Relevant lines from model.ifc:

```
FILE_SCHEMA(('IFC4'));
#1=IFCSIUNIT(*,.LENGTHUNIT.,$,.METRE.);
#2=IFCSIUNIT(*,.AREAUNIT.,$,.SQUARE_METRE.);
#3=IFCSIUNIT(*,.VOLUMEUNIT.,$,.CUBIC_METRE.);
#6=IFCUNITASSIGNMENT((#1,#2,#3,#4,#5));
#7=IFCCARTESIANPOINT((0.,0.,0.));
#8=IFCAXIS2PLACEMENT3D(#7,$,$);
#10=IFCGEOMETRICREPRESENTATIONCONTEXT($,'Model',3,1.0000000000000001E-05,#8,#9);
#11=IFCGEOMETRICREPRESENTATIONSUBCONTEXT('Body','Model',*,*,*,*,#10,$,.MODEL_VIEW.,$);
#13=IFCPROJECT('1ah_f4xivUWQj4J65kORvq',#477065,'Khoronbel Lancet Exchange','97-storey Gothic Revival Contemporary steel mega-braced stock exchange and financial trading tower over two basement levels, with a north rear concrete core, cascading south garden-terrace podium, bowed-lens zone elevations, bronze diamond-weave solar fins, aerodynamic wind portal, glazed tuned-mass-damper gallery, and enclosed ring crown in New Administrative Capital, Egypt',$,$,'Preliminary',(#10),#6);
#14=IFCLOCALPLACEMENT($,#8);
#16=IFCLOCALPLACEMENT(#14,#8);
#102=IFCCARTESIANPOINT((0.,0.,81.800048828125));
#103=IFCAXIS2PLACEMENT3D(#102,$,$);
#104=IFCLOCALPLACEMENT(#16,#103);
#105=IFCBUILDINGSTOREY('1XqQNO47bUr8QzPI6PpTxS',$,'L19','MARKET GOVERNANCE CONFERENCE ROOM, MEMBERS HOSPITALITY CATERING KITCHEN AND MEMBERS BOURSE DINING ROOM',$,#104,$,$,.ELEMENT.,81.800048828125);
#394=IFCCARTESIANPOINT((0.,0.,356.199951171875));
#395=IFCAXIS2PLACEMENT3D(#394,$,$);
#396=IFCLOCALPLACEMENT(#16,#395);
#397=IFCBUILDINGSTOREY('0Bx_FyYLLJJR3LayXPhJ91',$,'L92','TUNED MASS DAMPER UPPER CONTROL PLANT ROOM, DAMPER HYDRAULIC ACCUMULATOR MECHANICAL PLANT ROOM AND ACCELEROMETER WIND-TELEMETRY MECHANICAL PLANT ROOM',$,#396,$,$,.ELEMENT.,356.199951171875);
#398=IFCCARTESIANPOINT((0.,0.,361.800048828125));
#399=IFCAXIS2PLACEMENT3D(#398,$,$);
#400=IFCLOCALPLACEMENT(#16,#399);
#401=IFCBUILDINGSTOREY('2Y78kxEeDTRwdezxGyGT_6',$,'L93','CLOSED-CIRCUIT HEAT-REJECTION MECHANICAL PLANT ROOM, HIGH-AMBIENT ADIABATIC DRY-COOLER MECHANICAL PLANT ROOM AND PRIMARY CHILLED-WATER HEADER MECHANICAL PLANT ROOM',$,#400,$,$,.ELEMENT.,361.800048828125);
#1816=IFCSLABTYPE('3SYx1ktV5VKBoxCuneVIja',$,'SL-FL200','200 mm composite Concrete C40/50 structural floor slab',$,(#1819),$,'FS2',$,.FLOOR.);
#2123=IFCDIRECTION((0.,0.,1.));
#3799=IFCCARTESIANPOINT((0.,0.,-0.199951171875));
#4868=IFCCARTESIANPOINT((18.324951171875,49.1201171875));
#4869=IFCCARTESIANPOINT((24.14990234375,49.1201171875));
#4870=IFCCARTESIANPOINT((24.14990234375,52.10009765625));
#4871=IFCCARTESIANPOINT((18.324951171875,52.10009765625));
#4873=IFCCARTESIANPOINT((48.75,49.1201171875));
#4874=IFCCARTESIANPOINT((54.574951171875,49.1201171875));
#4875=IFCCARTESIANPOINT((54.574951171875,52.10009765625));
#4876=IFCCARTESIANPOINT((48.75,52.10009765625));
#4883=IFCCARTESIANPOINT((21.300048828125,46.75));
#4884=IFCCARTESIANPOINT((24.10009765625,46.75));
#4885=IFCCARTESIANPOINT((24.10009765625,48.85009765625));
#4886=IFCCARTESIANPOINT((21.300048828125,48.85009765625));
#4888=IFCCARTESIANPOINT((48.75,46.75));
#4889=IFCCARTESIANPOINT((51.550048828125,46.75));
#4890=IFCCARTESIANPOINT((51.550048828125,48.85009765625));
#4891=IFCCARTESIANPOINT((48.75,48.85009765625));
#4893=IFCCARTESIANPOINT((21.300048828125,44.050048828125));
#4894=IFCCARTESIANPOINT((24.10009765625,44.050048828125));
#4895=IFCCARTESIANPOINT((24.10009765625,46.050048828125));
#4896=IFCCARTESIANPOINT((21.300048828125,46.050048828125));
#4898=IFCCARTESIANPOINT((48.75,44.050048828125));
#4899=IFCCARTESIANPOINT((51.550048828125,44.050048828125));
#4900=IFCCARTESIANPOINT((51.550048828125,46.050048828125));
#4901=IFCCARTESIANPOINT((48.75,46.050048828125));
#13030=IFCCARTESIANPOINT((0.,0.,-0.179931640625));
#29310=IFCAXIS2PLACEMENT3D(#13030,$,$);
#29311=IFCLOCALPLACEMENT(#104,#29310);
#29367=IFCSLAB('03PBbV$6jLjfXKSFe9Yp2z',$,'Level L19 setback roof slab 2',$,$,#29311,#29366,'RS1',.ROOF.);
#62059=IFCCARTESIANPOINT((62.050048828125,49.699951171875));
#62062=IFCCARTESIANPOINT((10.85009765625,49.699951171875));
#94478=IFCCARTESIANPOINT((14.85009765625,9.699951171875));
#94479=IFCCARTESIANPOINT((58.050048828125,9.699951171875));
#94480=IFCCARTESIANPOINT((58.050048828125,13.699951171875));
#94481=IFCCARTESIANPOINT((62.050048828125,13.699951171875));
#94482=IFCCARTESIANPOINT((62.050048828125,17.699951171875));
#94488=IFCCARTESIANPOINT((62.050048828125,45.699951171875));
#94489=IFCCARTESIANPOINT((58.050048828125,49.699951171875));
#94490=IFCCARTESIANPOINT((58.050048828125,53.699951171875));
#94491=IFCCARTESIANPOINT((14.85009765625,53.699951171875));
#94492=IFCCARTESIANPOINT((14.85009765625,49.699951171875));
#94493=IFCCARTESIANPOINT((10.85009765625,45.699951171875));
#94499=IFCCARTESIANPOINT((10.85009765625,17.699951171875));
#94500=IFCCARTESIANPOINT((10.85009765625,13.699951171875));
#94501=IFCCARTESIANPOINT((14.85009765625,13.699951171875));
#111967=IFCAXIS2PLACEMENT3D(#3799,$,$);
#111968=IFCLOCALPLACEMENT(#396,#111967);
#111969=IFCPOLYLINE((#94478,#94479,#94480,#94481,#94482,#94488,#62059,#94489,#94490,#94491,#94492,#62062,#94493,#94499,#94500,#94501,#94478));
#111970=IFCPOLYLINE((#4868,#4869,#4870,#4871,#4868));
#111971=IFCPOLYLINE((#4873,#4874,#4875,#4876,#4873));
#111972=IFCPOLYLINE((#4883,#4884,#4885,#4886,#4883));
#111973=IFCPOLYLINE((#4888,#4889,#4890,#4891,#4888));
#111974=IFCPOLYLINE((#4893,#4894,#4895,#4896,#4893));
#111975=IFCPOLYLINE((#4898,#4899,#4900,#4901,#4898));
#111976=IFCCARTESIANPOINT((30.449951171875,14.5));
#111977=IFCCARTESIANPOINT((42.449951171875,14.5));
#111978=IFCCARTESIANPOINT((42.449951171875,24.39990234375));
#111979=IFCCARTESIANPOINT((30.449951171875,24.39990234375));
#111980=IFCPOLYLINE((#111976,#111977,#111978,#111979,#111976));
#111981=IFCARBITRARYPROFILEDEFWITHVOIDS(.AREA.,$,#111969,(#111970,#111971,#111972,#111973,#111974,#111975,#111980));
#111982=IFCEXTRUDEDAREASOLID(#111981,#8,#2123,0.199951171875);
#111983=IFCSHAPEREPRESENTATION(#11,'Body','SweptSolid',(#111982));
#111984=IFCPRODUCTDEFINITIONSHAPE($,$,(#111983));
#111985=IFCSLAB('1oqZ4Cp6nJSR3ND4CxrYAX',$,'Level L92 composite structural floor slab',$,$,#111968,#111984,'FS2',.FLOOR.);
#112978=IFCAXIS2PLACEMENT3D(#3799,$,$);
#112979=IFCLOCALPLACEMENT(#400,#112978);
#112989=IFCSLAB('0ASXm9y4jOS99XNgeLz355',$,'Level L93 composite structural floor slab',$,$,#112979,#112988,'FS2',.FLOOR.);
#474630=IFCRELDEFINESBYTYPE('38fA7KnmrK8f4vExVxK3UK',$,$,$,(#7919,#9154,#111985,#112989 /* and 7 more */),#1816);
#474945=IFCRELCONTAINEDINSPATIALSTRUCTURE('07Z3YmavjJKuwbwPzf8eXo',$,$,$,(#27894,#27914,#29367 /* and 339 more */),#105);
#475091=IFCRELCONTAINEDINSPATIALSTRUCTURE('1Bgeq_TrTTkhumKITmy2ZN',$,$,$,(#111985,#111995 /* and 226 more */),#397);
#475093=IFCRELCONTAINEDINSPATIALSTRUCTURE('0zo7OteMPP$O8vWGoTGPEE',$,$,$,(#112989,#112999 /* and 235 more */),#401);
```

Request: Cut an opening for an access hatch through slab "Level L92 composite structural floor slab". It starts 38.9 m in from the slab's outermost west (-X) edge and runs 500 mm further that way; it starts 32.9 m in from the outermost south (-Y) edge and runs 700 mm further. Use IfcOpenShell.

```python
import numpy as np
import ifcopenshell
import ifcopenshell.api.feature
import ifcopenshell.api.geometry
import ifcopenshell.api.root
import ifcopenshell.geom
import ifcopenshell.util.placement
import ifcopenshell.util.representation
import ifcopenshell.util.shape
import ifcopenshell.util.unit

model = ifcopenshell.open("model.ifc")
unit_scale = ifcopenshell.util.unit.calculate_unit_scale(model)
settings = ifcopenshell.geom.settings()


def volume(element):
    """Net volume in cubic metres, openings subtracted."""
    shape = ifcopenshell.geom.create_shape(settings, element)
    return ifcopenshell.util.shape.get_volume(shape.geometry)


slab = model.by_guid("1oqZ4Cp6nJSR3ND4CxrYAX")
before = volume(slab)

# Extent in the slab's own axes, in metres. The edges named are its -X and -Y sides.
slab_shape = ifcopenshell.geom.create_shape(settings, slab)
vertices = ifcopenshell.util.shape.get_vertices(slab_shape.geometry)
x_min, y_min, bottom = vertices.min(axis=0)
top = vertices[:, 2].max()

opening = ifcopenshell.api.root.create_entity(model, ifc_class="IfcOpeningElement", name="Access hatch opening", predefined_type="OPENING")
context = ifcopenshell.util.representation.get_context(model, "Model", "Body", "MODEL_VIEW")
width, depth = 0.5, 0.7
outline = [(0.0, 0.0), (width, 0.0), (width, depth), (0.0, depth), (0.0, 0.0)]
# Overshoot both faces by 50 mm so the cut is clean.
shape = ifcopenshell.api.geometry.add_slab_representation(
    model, context=context, depth=top - bottom + 0.1, polyline=outline
)
ifcopenshell.api.geometry.assign_representation(model, product=opening, representation=shape)

matrix = ifcopenshell.util.placement.get_local_placement(slab.ObjectPlacement)
matrix[:, 3] = matrix @ np.append(np.array([x_min + 38.9, y_min + 32.9, bottom - 0.05]) / unit_scale, 1.0)
ifcopenshell.api.geometry.edit_object_placement(model, product=opening, matrix=matrix, is_si=False)
ifcopenshell.api.feature.add_feature(model, feature=opening, element=slab)

after = volume(slab)

print(f"slab volume {before:.3f} -> {after:.3f} m3")

model.write("model_rev.ifc")
```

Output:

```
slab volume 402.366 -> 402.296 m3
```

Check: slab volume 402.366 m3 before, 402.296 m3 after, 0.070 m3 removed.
